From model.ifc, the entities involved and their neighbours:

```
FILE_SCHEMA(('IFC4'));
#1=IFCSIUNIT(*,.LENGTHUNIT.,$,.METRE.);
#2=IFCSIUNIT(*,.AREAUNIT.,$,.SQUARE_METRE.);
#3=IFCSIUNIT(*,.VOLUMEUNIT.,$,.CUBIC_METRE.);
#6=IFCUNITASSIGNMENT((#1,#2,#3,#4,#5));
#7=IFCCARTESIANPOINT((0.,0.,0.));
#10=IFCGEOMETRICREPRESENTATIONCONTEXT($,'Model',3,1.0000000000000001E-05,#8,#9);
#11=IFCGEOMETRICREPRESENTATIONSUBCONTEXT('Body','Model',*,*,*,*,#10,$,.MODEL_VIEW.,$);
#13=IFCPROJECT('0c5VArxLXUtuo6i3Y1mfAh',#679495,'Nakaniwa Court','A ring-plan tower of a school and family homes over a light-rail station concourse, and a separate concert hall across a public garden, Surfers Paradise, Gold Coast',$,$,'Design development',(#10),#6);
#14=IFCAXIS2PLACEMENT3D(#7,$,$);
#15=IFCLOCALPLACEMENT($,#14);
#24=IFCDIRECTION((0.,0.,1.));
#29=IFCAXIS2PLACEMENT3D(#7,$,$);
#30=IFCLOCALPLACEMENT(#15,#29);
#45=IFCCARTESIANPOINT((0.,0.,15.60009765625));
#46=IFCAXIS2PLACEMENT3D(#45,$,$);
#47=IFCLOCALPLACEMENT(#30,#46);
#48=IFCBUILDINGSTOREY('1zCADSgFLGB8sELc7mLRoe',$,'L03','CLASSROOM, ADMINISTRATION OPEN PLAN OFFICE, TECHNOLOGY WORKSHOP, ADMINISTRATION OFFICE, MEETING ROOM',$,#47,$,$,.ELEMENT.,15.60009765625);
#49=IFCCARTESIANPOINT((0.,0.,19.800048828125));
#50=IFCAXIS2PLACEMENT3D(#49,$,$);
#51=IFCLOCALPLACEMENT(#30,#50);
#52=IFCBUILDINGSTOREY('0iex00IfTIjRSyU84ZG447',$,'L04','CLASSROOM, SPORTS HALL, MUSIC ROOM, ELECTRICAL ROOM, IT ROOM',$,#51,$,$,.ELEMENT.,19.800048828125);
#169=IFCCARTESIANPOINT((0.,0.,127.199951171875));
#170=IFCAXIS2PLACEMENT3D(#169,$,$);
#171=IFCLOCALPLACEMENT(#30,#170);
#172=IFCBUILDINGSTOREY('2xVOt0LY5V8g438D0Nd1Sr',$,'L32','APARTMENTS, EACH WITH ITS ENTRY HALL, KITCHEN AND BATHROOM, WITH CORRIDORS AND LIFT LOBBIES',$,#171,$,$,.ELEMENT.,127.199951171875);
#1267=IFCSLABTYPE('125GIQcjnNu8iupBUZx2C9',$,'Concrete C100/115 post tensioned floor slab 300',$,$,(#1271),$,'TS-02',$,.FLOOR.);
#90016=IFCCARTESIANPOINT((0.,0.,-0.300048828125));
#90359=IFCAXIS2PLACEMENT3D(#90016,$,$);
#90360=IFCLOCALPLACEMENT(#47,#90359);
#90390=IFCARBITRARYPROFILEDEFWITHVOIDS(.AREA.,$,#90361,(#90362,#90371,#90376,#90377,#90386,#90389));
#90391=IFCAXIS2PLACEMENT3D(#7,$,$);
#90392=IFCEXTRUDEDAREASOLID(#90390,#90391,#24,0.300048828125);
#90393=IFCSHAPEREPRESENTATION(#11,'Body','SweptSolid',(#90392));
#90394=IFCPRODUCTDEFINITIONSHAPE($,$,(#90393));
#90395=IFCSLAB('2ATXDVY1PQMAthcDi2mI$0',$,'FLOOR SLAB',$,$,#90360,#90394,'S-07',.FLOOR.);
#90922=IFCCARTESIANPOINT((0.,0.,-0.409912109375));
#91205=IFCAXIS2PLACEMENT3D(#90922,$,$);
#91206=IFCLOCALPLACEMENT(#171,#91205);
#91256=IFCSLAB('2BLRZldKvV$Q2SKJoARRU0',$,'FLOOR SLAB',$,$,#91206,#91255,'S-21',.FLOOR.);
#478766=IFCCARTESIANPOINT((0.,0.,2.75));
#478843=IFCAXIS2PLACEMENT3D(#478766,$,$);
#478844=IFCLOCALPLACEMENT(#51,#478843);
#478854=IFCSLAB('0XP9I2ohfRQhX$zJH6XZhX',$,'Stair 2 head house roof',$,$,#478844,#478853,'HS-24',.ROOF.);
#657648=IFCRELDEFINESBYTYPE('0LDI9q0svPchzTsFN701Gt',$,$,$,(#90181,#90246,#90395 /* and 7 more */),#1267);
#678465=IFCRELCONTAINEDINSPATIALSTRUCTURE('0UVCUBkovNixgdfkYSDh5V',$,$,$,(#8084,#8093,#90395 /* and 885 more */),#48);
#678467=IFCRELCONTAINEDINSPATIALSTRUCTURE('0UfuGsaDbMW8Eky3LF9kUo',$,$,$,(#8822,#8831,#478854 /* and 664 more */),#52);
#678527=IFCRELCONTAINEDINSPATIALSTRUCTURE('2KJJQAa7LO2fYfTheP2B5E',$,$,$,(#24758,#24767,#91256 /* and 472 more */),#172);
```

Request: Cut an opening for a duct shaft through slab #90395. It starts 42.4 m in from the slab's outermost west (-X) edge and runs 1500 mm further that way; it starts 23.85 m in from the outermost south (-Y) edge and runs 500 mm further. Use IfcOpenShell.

```python
import numpy as np
import ifcopenshell
import ifcopenshell.api.feature
import ifcopenshell.api.geometry
import ifcopenshell.api.root
import ifcopenshell.geom
import ifcopenshell.util.placement
import ifcopenshell.util.representation
import ifcopenshell.util.shape
import ifcopenshell.util.unit

model = ifcopenshell.open("model.ifc")
unit_scale = ifcopenshell.util.unit.calculate_unit_scale(model)
settings = ifcopenshell.geom.settings()


def volume(element):
    """Net volume in cubic metres, openings subtracted."""
    shape = ifcopenshell.geom.create_shape(settings, element)
    return ifcopenshell.util.shape.get_volume(shape.geometry)


slab = model.by_guid("2ATXDVY1PQMAthcDi2mI$0")
before = volume(slab)

# Extent in the slab's own axes, in metres. The edges named are its -X and -Y sides.
slab_shape = ifcopenshell.geom.create_shape(settings, slab)
vertices = ifcopenshell.util.shape.get_vertices(slab_shape.geometry)
x_min, y_min, bottom = vertices.min(axis=0)
top = vertices[:, 2].max()

opening = ifcopenshell.api.root.create_entity(model, ifc_class="IfcOpeningElement", name="Duct shaft opening", predefined_type="OPENING")
context = ifcopenshell.util.representation.get_context(model, "Model", "Body", "MODEL_VIEW")
width, depth = 1.5, 0.5
outline = [(0.0, 0.0), (width, 0.0), (width, depth), (0.0, depth), (0.0, 0.0)]
# Overshoot both faces by 50 mm so the cut is clean.
shape = ifcopenshell.api.geometry.add_slab_representation(
    model, context=context, depth=top - bottom + 0.1, polyline=outline
)
ifcopenshell.api.geometry.assign_representation(model, product=opening, representation=shape)

matrix = ifcopenshell.util.placement.get_local_placement(slab.ObjectPlacement)
matrix[:, 3] = matrix @ np.append(np.array([x_min + 42.4, y_min + 23.85, bottom - 0.05]) / unit_scale, 1.0)
ifcopenshell.api.geometry.edit_object_placement(model, product=opening, matrix=matrix, is_si=False)
ifcopenshell.api.feature.add_feature(model, feature=opening, element=slab)

after = volume(slab)

print(f"slab volume {before:.3f} -> {after:.3f} m3")

model.write("model_v2.ifc")
```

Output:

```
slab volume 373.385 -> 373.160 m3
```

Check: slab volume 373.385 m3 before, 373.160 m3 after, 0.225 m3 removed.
